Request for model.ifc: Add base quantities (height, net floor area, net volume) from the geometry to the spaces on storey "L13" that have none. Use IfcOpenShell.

First a look at what the model holds.

```python
import ifcopenshell
import ifcopenshell.util.element
import ifcopenshell.util.unit

model = ifcopenshell.open("model.ifc")
print(model.schema)
for unit_type in ("LENGTHUNIT", "AREAUNIT", "VOLUMEUNIT"):
    print(unit_type, ifcopenshell.util.unit.calculate_unit_scale(model, unit_type))
storey = next(s for s in model.by_type("IfcBuildingStorey") if s.Name == "L13")
spaces = [e for e in ifcopenshell.util.element.get_decomposition(storey) if e.is_a("IfcSpace")]
for e in sorted(spaces, key=lambda e: e.id()):
    print(e.id(), e.is_a(), e.Name, list(ifcopenshell.util.element.get_psets(e, qtos_only=True)), sep=" | ")
```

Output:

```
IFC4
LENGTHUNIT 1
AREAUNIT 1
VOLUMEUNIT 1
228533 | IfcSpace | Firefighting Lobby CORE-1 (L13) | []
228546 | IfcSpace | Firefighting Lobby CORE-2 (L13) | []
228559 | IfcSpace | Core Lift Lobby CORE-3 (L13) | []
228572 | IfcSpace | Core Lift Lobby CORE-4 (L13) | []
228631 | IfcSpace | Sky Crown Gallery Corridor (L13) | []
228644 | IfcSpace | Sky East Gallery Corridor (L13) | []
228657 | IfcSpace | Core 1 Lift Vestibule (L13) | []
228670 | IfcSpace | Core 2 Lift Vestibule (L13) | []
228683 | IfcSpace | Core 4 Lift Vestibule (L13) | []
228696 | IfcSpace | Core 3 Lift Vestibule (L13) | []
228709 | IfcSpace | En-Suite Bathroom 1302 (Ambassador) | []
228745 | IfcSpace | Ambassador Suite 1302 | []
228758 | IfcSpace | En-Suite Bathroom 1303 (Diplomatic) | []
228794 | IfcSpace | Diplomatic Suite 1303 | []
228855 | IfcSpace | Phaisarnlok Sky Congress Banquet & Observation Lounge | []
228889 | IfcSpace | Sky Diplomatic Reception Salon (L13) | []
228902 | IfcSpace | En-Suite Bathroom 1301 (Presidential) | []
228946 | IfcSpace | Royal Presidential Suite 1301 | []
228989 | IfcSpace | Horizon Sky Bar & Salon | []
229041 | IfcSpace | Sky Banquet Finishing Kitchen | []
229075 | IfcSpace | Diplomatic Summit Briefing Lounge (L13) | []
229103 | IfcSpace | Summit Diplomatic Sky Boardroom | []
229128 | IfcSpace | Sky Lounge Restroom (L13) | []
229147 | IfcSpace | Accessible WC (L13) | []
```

```python
import ifcopenshell
import ifcopenshell.api.pset
import ifcopenshell.geom
import ifcopenshell.util.element
import ifcopenshell.util.shape
import ifcopenshell.util.unit

model = ifcopenshell.open("model.ifc")
unit_scale = ifcopenshell.util.unit.calculate_unit_scale(model)
area_scale = ifcopenshell.util.unit.calculate_unit_scale(model, "AREAUNIT")
volume_scale = ifcopenshell.util.unit.calculate_unit_scale(model, "VOLUMEUNIT")
settings = ifcopenshell.geom.settings()

storey = next(s for s in model.by_type("IfcBuildingStorey") if s.Name == "L13")
spaces = [e for e in ifcopenshell.util.element.get_decomposition(storey) if e.is_a("IfcSpace")]

for e in sorted(spaces, key=lambda e: e.id()):
    if ifcopenshell.util.element.get_psets(e, qtos_only=True, should_inherit=False):
        continue
    # Geometry comes back in metres, in the element's own axes.
    shape = ifcopenshell.geom.create_shape(settings, e)
    values = {
        "Height": ifcopenshell.util.shape.get_z(shape.geometry) / unit_scale,
        "NetFloorArea": ifcopenshell.util.shape.get_footprint_area(shape.geometry) / area_scale,
        "NetVolume": ifcopenshell.util.shape.get_volume(shape.geometry) / volume_scale,
    }
    qto = ifcopenshell.api.pset.add_qto(model, product=e, name="Qto_SpaceBaseQuantities")
    ifcopenshell.api.pset.edit_qto(model, qto=qto, properties=values)
    print(e.id(), {k: round(v, 3) for k, v in values.items()})

model.write("model_v2.ifc")
```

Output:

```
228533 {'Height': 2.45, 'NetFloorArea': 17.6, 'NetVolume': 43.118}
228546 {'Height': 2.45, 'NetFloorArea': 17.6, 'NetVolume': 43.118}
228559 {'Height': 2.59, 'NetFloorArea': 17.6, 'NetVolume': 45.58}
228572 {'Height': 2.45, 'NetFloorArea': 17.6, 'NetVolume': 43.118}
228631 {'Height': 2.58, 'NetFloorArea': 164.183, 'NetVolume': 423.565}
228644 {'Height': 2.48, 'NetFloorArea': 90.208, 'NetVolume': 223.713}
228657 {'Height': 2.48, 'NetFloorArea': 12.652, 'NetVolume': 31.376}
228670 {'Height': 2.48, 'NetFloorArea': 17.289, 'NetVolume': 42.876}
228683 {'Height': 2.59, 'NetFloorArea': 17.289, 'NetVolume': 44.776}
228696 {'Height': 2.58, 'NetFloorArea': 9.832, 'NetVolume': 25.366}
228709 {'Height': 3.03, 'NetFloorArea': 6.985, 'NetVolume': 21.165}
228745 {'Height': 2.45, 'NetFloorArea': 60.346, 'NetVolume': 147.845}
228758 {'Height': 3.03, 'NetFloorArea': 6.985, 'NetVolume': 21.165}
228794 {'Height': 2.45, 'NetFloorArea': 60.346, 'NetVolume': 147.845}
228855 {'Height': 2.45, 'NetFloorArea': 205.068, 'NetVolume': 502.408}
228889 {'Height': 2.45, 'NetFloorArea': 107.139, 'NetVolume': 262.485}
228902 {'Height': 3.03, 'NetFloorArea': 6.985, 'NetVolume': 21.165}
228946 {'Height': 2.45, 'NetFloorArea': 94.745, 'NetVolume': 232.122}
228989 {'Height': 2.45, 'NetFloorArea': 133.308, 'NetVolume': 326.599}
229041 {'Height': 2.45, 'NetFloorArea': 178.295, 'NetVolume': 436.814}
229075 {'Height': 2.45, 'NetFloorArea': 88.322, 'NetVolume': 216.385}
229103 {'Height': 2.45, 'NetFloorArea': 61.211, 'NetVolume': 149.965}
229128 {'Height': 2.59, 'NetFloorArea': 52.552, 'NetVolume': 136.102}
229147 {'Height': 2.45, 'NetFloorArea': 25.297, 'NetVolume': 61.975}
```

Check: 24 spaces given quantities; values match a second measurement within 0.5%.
